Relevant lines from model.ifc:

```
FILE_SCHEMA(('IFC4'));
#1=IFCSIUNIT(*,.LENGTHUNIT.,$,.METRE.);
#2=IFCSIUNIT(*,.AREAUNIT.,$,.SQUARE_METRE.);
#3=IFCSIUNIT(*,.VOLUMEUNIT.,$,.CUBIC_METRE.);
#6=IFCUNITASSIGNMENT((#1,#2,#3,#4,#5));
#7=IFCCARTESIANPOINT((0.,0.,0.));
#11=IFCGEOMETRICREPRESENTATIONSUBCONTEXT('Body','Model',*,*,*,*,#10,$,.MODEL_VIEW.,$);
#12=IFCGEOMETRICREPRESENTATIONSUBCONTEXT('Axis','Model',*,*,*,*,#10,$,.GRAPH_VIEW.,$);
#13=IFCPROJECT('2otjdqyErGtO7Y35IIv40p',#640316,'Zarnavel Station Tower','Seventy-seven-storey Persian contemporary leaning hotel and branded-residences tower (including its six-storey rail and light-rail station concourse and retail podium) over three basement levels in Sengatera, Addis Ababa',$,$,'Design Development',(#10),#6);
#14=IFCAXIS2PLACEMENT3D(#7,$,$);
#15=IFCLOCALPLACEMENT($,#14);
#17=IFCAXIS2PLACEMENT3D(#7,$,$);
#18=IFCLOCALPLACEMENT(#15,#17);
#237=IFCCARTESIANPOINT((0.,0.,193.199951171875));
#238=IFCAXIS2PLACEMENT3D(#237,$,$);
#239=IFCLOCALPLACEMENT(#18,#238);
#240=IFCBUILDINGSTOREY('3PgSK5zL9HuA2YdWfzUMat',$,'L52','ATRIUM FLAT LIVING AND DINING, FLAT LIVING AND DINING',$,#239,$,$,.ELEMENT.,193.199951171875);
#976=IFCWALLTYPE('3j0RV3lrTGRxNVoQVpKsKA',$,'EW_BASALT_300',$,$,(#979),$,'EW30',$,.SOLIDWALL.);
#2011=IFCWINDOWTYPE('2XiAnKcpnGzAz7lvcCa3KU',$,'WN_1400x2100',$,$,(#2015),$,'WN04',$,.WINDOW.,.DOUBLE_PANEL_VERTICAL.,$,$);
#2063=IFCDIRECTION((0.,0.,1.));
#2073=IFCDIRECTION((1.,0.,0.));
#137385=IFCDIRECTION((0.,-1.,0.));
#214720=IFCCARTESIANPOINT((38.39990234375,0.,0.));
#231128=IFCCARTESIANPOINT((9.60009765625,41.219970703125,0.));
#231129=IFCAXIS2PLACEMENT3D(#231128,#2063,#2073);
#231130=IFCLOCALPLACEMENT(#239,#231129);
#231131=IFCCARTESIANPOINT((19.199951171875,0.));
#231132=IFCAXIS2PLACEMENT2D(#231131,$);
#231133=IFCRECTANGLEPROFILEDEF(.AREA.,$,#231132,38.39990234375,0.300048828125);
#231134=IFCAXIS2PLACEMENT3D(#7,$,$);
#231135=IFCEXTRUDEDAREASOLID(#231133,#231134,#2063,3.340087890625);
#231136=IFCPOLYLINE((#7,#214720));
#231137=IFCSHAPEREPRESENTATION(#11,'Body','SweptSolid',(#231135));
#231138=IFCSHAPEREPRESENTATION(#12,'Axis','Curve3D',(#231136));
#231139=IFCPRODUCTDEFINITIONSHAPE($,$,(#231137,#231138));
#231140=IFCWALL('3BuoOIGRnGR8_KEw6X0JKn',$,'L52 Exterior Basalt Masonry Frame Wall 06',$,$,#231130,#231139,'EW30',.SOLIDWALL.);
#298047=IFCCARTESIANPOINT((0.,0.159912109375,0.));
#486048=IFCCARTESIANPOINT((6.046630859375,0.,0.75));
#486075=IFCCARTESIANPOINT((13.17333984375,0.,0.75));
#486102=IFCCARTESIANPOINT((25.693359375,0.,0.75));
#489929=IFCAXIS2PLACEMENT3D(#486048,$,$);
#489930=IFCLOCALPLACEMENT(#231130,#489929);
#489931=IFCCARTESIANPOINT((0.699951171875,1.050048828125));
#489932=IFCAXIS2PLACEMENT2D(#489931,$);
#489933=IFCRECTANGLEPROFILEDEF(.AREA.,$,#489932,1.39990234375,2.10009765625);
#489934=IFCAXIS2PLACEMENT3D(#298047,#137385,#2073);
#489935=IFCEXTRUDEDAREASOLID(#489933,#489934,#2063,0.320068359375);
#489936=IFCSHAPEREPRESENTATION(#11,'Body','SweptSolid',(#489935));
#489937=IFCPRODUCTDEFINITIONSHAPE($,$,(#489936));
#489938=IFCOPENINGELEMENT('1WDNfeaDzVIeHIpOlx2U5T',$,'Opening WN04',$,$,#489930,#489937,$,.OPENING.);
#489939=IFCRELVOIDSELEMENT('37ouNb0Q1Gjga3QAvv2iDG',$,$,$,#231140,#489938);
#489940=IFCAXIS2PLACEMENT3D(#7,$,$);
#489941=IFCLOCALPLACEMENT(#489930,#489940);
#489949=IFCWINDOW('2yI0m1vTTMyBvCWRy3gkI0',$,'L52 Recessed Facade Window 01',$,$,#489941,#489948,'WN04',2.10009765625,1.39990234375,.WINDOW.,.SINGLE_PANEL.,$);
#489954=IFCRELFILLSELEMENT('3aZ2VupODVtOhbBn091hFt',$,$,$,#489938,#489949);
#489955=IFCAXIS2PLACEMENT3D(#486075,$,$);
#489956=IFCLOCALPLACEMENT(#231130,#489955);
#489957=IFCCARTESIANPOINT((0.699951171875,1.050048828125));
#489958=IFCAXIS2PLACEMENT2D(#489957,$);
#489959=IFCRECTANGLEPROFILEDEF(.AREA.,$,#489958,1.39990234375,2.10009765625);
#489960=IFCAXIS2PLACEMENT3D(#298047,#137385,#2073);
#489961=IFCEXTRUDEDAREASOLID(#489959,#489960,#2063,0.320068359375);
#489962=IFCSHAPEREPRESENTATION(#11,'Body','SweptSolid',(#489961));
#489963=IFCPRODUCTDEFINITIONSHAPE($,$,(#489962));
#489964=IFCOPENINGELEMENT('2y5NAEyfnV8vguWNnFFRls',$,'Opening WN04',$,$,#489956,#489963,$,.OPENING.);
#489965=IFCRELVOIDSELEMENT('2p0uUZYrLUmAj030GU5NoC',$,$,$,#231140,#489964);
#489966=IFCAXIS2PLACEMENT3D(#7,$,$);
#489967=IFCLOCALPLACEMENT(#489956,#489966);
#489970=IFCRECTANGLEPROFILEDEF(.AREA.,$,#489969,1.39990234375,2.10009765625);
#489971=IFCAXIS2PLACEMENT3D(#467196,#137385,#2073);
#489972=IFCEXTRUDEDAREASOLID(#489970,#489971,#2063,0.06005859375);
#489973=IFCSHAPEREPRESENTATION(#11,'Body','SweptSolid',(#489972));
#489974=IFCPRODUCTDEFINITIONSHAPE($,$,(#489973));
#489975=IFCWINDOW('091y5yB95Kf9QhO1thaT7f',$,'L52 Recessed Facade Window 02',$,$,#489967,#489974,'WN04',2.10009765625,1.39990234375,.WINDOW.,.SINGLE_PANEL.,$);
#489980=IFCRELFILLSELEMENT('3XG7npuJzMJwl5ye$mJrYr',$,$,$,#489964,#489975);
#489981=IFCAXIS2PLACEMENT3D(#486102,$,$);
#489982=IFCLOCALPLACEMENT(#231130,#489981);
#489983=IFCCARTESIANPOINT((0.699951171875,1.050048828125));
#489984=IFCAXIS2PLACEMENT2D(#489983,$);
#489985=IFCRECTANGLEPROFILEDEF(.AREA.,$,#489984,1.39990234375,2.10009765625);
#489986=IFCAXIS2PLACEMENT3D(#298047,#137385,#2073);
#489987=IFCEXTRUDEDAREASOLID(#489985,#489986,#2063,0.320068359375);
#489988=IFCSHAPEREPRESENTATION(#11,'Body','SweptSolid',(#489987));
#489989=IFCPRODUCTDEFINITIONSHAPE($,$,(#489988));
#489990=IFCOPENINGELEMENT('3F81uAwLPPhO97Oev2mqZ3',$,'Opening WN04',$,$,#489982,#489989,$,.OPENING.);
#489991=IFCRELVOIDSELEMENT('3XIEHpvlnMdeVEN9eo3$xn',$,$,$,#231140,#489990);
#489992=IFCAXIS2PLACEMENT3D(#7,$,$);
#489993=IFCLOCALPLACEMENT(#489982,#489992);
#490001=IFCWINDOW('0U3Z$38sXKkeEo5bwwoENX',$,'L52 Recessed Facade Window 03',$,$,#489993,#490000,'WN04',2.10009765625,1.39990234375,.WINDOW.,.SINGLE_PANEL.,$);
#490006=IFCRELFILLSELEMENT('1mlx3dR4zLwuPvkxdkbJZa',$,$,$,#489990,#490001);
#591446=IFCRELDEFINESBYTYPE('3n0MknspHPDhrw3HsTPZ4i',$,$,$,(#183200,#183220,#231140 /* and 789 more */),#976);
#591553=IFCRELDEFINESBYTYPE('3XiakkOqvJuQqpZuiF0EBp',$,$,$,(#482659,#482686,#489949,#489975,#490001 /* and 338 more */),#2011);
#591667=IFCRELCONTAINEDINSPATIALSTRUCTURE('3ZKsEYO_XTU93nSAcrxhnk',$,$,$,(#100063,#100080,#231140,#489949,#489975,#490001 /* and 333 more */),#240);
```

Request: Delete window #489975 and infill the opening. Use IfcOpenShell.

```python
import ifcopenshell
import ifcopenshell.api.feature
import ifcopenshell.api.root
import ifcopenshell.geom
import ifcopenshell.util.shape

model = ifcopenshell.open("model.ifc")
settings = ifcopenshell.geom.settings()


def volume(element):
    """Net volume in cubic metres, openings subtracted."""
    shape = ifcopenshell.geom.create_shape(settings, element)
    return ifcopenshell.util.shape.get_volume(shape.geometry)


window = model.by_guid("091y5yB95Kf9QhO1thaT7f")
opening = window.FillsVoids[0].RelatingOpeningElement
wall = opening.VoidsElements[0].RelatingBuildingElement
before = volume(wall)

ifcopenshell.api.root.remove_product(model, product=window)
ifcopenshell.api.feature.remove_feature(model, feature=opening)

after = volume(wall)

print(f"wall volume {before:.3f} -> {after:.3f} m3")

model.write("model_v2.ifc")
```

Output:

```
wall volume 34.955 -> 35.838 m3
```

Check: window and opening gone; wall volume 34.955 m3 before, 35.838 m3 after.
